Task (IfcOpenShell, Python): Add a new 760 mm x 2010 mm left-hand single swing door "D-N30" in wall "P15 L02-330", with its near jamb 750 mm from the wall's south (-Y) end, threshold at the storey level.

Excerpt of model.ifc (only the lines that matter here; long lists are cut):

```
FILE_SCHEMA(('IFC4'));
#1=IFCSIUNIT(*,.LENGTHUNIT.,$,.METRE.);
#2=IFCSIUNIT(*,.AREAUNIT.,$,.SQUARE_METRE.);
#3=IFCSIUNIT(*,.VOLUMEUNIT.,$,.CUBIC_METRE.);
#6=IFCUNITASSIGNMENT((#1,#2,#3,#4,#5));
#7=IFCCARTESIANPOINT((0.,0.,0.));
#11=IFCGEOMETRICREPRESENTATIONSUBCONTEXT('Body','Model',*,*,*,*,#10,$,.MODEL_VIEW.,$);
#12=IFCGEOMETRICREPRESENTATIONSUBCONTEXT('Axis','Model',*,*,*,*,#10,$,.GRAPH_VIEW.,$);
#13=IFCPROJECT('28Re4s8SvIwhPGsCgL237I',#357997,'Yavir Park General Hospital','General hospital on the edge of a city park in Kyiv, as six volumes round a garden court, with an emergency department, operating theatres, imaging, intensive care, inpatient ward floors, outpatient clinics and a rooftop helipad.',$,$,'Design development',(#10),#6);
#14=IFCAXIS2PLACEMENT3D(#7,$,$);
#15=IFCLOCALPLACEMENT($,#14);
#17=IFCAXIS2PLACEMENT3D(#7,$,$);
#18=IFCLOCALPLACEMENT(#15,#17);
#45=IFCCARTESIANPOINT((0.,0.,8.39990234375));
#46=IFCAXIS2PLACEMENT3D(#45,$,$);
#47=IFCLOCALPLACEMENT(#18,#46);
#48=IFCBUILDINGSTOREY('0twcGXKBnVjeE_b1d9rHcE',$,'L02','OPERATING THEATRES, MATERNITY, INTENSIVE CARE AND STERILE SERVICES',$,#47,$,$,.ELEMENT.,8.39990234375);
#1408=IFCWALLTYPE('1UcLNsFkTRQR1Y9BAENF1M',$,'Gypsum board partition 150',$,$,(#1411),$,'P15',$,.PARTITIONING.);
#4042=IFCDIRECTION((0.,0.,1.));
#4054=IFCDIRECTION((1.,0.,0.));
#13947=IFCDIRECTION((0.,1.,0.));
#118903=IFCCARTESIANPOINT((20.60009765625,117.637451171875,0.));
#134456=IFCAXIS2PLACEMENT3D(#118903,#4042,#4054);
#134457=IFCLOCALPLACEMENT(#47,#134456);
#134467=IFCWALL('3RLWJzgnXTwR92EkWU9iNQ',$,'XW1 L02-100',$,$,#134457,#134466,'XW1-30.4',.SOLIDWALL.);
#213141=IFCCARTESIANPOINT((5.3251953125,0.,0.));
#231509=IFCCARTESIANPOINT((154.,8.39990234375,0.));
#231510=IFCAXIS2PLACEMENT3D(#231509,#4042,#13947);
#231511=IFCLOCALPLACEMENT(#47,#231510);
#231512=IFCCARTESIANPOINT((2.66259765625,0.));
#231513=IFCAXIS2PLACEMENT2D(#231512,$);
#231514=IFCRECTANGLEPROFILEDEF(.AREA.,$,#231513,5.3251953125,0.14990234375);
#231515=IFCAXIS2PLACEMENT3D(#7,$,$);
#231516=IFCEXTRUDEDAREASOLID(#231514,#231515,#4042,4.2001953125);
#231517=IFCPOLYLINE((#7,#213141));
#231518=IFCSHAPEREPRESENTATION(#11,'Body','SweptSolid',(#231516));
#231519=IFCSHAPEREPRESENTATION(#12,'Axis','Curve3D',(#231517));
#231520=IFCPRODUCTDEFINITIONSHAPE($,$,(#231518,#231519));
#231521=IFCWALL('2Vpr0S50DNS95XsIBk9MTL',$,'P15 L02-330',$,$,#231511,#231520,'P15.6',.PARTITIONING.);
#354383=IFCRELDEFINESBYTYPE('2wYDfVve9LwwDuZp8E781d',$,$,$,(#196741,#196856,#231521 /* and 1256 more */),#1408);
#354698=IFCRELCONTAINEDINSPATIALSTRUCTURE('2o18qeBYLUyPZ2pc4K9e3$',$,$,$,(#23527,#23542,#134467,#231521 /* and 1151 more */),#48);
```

```python
import numpy as np
import ifcopenshell
import ifcopenshell.api.feature
import ifcopenshell.api.geometry
import ifcopenshell.api.root
import ifcopenshell.api.spatial
import ifcopenshell.geom
import ifcopenshell.util.element
import ifcopenshell.util.placement
import ifcopenshell.util.representation
import ifcopenshell.util.shape
import ifcopenshell.util.unit

model = ifcopenshell.open("model.ifc")
unit_scale = ifcopenshell.util.unit.calculate_unit_scale(model)
settings = ifcopenshell.geom.settings()


def volume(element):
    """Net volume in cubic metres, openings subtracted."""
    shape = ifcopenshell.geom.create_shape(settings, element)
    return ifcopenshell.util.shape.get_volume(shape.geometry)


wall = model.by_guid("2Vpr0S50DNS95XsIBk9MTL")
storey = ifcopenshell.util.element.get_container(wall, ifc_class="IfcBuildingStorey")
context = ifcopenshell.util.representation.get_context(model, "Model", "Body", "MODEL_VIEW")
before = volume(wall)

width, height, from_end, sill = 0.76, 2.01, 0.75, 0.0  # metres

# The wall runs along its own X axis, and the end named is its -X end.
wall_shape = ifcopenshell.geom.create_shape(settings, wall)
x, y, z = ifcopenshell.util.shape.get_vertices(wall_shape.geometry).T
start = x.min() + from_end
face, thickness = float(y.min()), float(y.max() - y.min())
wall_matrix = ifcopenshell.util.placement.get_local_placement(wall.ObjectPlacement)
level = ifcopenshell.util.placement.get_local_placement(storey.ObjectPlacement)[2, 3]


def in_wall(x, y):
    """Placement at x, y metres in the wall's axes, at sill height."""
    matrix = wall_matrix.copy()
    matrix[:, 3] = wall_matrix @ np.array([x / unit_scale, y / unit_scale, 0.0, 1.0])
    matrix[2, 3] = level + sill / unit_scale
    return matrix


# Opening: a box that overshoots both wall faces by 50 mm.
opening = ifcopenshell.api.root.create_entity(model, ifc_class="IfcOpeningElement", predefined_type="OPENING")
box = ifcopenshell.api.geometry.add_wall_representation(
    model, context=context, length=width, height=height, thickness=thickness + 0.1
)
ifcopenshell.api.geometry.assign_representation(model, product=opening, representation=box)
ifcopenshell.api.geometry.edit_object_placement(model, product=opening, matrix=in_wall(start, face - 0.05), is_si=False)
ifcopenshell.api.feature.add_feature(model, feature=opening, element=wall)

door = ifcopenshell.api.root.create_entity(model, ifc_class="IfcDoor", name="D-N30", predefined_type="DOOR")
door.OverallWidth, door.OverallHeight = width / unit_scale, height / unit_scale
door.OperationType = "SINGLE_SWING_LEFT"
body = ifcopenshell.api.geometry.add_door_representation(
    model,
    context=context,
    overall_width=door.OverallWidth,
    overall_height=door.OverallHeight,
    operation_type="SINGLE_SWING_LEFT",
    lining_properties={"LiningDepth": thickness / unit_scale, "ThresholdDepth": thickness / unit_scale},
)
ifcopenshell.api.geometry.assign_representation(model, product=door, representation=body)
ifcopenshell.api.spatial.assign_container(model, products=[door], relating_structure=storey)
ifcopenshell.api.feature.add_filling(model, opening=opening, element=door)

# The lining spans the wall, so the door starts at the wall face.
ifcopenshell.api.geometry.edit_object_placement(model, product=door, matrix=in_wall(start, face), is_si=False)

after = volume(wall)

print(f"wall volume {before:.3f} -> {after:.3f} m3")

model.write("model_edited.ifc")
```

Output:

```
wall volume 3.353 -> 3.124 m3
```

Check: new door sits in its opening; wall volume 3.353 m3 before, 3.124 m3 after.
